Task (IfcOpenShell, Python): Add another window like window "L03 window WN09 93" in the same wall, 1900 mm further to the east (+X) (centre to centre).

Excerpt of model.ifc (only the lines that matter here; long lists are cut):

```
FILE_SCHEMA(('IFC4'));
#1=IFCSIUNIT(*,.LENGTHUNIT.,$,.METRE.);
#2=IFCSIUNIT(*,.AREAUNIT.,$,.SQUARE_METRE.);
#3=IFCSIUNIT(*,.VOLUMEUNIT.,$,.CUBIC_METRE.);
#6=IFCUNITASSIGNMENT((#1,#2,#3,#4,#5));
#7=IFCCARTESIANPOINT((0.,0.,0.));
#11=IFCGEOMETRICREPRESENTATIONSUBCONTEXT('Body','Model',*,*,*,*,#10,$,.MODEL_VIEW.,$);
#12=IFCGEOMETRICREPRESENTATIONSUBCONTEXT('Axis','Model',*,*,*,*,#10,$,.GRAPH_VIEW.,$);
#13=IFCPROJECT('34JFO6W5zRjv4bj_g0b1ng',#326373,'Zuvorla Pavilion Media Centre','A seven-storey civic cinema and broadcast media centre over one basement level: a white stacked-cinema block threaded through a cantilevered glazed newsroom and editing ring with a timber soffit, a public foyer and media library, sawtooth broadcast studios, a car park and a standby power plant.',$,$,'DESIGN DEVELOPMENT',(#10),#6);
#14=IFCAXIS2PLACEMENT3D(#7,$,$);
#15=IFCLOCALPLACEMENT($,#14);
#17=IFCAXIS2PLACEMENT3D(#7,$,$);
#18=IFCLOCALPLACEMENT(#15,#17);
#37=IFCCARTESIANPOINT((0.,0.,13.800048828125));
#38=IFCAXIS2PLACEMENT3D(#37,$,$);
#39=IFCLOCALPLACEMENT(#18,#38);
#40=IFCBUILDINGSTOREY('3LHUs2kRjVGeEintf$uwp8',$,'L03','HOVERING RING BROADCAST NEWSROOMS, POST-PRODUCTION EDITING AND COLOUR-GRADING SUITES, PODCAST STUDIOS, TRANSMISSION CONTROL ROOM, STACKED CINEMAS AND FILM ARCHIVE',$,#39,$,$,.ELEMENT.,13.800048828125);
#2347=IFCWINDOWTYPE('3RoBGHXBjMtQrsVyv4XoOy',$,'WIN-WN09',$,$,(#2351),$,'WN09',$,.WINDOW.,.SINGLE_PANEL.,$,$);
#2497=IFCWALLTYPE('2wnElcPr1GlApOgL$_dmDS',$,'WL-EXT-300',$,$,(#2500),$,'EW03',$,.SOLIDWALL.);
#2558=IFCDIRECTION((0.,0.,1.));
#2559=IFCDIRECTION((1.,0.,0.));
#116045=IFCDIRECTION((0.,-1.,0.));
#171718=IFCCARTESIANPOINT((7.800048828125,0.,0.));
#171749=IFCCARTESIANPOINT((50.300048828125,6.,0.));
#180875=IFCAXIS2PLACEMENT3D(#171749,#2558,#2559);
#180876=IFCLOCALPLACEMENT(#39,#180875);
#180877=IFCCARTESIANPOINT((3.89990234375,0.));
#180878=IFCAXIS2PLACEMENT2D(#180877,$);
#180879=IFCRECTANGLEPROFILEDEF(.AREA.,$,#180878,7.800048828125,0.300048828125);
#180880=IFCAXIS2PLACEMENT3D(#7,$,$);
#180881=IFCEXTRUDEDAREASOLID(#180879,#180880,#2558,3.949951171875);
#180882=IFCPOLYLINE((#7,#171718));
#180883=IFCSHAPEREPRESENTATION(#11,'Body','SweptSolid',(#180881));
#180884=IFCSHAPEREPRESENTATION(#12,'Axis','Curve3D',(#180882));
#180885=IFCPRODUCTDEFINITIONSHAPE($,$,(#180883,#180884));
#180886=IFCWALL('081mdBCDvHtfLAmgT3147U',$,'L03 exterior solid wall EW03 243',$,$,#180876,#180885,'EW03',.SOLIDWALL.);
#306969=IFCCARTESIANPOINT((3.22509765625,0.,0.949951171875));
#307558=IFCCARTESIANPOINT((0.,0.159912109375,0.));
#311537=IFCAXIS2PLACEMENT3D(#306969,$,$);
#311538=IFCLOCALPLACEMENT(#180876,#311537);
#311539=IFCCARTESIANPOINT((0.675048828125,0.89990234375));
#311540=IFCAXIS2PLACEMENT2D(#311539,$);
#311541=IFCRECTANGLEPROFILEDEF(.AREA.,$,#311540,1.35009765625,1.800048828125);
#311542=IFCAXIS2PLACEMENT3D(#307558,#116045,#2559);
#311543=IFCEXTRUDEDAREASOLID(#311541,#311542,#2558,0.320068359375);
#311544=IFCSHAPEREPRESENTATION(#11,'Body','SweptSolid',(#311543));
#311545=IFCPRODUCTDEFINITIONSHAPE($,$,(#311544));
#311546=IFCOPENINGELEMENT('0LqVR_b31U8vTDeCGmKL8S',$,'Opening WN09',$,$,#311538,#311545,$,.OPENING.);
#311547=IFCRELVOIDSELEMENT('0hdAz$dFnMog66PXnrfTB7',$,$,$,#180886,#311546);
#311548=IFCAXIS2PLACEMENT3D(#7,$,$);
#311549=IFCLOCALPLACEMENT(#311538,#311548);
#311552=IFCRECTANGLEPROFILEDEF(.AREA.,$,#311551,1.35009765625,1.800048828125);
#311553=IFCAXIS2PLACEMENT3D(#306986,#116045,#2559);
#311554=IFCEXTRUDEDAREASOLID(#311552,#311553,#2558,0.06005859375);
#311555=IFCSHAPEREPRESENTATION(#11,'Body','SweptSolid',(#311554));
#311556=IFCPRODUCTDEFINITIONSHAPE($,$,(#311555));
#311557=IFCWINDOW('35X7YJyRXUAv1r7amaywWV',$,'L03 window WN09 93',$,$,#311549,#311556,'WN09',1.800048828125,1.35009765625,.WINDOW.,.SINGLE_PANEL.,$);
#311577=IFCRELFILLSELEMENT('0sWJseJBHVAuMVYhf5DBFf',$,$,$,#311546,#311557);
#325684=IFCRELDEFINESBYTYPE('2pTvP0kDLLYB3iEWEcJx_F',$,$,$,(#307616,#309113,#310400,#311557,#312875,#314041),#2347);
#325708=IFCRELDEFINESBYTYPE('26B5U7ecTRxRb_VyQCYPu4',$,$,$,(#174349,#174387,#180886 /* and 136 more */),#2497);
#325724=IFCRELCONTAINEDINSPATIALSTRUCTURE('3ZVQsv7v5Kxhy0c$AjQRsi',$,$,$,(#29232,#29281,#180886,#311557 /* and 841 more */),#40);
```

```python
import ifcopenshell
import ifcopenshell.api.feature
import ifcopenshell.api.geometry
import ifcopenshell.api.root
import ifcopenshell.geom
import ifcopenshell.util.element
import ifcopenshell.util.placement
import ifcopenshell.util.shape
import ifcopenshell.util.unit

model = ifcopenshell.open("model.ifc")
unit_scale = ifcopenshell.util.unit.calculate_unit_scale(model)
settings = ifcopenshell.geom.settings()


def volume(element):
    """Net volume in cubic metres, openings subtracted."""
    shape = ifcopenshell.geom.create_shape(settings, element)
    return ifcopenshell.util.shape.get_volume(shape.geometry)


window = model.by_guid("35X7YJyRXUAv1r7amaywWV")
opening = window.FillsVoids[0].RelatingOpeningElement
wall = opening.VoidsElements[0].RelatingBuildingElement
before = volume(wall)
shift = ifcopenshell.util.placement.get_local_placement(wall.ObjectPlacement)[:3, 0] * 1.9 / unit_scale

# copy_class copies the void relationship, type, container and properties, but no geometry.
new_opening = ifcopenshell.api.root.copy_class(model, product=opening)
new_opening.Representation = ifcopenshell.util.element.copy_deep(
    model, opening.Representation, exclude=["IfcGeometricRepresentationContext", "IfcRepresentationMap"]
)
new_window = ifcopenshell.api.root.copy_class(model, product=window)
new_window.Representation = ifcopenshell.util.element.copy_deep(
    model, window.Representation, exclude=["IfcGeometricRepresentationContext", "IfcRepresentationMap"]
)
new_window.Tag = None
ifcopenshell.api.feature.add_filling(model, opening=new_opening, element=new_window)

for old, new in ((opening, new_opening), (window, new_window)):
    matrix = ifcopenshell.util.placement.get_local_placement(old.ObjectPlacement)
    matrix[:3, 3] += shift
    ifcopenshell.api.geometry.edit_object_placement(model, product=new, matrix=matrix, is_si=False)

after = volume(wall)

print(f"wall volume {before:.3f} -> {after:.3f} m3")

model.write("model_edited.ifc")
```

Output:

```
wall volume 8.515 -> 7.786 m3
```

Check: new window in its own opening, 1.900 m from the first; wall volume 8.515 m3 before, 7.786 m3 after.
